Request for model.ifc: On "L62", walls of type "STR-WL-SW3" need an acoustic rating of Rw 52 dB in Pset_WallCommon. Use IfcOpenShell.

First a look at what the model holds.

```python
import ifcopenshell
import ifcopenshell.util.element

model = ifcopenshell.open("model.ifc")
print(model.schema)
storey = next(s for s in model.by_type("IfcBuildingStorey") if s.Name == "L62")
walls = [e for e in ifcopenshell.util.element.get_decomposition(storey) if e.is_a("IfcWall")]
seen = {}
for e in walls:
    element_type = ifcopenshell.util.element.get_type(e)
    key = (element_type.Name if element_type != e and element_type else None, ifcopenshell.util.element.get_pset(e, "Pset_WallCommon", "AcousticRating"))
    seen[key] = seen.get(key, 0) + 1
for (name, value), count in sorted(seen.items(), key=str):
    print(count, "x", name, "|", value)
```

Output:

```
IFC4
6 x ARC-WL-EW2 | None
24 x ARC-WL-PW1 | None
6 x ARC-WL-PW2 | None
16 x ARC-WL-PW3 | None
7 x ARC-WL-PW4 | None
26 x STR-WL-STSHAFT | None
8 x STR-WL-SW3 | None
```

```python
import ifcopenshell
import ifcopenshell.api.pset
import ifcopenshell.util.element

model = ifcopenshell.open("model.ifc")

storey = next(s for s in model.by_type("IfcBuildingStorey") if s.Name == "L62")
walls = [e for e in ifcopenshell.util.element.get_decomposition(storey) if e.is_a("IfcWall")]

count = 0
for e in walls:
    element_type = ifcopenshell.util.element.get_type(e)
    if element_type in (None, e) or element_type.Name != "STR-WL-SW3":
        continue
    found = ifcopenshell.util.element.get_pset(e, "Pset_WallCommon", should_inherit=False)
    if found:
        pset = model.by_id(found["id"])
        if len(ifcopenshell.util.element.get_elements_by_pset(pset)) > 1:
            pset = ifcopenshell.api.pset.unshare_pset(model, products=[e], pset=pset)[0]
    else:
        pset = ifcopenshell.api.pset.add_pset(model, product=e, name="Pset_WallCommon")
    ifcopenshell.api.pset.edit_pset(model, pset=pset, properties={"AcousticRating": "Rw 52 dB"})
    count += 1

print(count, "walls updated")

model.write("model_edited.ifc")
```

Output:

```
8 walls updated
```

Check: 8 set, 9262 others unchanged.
